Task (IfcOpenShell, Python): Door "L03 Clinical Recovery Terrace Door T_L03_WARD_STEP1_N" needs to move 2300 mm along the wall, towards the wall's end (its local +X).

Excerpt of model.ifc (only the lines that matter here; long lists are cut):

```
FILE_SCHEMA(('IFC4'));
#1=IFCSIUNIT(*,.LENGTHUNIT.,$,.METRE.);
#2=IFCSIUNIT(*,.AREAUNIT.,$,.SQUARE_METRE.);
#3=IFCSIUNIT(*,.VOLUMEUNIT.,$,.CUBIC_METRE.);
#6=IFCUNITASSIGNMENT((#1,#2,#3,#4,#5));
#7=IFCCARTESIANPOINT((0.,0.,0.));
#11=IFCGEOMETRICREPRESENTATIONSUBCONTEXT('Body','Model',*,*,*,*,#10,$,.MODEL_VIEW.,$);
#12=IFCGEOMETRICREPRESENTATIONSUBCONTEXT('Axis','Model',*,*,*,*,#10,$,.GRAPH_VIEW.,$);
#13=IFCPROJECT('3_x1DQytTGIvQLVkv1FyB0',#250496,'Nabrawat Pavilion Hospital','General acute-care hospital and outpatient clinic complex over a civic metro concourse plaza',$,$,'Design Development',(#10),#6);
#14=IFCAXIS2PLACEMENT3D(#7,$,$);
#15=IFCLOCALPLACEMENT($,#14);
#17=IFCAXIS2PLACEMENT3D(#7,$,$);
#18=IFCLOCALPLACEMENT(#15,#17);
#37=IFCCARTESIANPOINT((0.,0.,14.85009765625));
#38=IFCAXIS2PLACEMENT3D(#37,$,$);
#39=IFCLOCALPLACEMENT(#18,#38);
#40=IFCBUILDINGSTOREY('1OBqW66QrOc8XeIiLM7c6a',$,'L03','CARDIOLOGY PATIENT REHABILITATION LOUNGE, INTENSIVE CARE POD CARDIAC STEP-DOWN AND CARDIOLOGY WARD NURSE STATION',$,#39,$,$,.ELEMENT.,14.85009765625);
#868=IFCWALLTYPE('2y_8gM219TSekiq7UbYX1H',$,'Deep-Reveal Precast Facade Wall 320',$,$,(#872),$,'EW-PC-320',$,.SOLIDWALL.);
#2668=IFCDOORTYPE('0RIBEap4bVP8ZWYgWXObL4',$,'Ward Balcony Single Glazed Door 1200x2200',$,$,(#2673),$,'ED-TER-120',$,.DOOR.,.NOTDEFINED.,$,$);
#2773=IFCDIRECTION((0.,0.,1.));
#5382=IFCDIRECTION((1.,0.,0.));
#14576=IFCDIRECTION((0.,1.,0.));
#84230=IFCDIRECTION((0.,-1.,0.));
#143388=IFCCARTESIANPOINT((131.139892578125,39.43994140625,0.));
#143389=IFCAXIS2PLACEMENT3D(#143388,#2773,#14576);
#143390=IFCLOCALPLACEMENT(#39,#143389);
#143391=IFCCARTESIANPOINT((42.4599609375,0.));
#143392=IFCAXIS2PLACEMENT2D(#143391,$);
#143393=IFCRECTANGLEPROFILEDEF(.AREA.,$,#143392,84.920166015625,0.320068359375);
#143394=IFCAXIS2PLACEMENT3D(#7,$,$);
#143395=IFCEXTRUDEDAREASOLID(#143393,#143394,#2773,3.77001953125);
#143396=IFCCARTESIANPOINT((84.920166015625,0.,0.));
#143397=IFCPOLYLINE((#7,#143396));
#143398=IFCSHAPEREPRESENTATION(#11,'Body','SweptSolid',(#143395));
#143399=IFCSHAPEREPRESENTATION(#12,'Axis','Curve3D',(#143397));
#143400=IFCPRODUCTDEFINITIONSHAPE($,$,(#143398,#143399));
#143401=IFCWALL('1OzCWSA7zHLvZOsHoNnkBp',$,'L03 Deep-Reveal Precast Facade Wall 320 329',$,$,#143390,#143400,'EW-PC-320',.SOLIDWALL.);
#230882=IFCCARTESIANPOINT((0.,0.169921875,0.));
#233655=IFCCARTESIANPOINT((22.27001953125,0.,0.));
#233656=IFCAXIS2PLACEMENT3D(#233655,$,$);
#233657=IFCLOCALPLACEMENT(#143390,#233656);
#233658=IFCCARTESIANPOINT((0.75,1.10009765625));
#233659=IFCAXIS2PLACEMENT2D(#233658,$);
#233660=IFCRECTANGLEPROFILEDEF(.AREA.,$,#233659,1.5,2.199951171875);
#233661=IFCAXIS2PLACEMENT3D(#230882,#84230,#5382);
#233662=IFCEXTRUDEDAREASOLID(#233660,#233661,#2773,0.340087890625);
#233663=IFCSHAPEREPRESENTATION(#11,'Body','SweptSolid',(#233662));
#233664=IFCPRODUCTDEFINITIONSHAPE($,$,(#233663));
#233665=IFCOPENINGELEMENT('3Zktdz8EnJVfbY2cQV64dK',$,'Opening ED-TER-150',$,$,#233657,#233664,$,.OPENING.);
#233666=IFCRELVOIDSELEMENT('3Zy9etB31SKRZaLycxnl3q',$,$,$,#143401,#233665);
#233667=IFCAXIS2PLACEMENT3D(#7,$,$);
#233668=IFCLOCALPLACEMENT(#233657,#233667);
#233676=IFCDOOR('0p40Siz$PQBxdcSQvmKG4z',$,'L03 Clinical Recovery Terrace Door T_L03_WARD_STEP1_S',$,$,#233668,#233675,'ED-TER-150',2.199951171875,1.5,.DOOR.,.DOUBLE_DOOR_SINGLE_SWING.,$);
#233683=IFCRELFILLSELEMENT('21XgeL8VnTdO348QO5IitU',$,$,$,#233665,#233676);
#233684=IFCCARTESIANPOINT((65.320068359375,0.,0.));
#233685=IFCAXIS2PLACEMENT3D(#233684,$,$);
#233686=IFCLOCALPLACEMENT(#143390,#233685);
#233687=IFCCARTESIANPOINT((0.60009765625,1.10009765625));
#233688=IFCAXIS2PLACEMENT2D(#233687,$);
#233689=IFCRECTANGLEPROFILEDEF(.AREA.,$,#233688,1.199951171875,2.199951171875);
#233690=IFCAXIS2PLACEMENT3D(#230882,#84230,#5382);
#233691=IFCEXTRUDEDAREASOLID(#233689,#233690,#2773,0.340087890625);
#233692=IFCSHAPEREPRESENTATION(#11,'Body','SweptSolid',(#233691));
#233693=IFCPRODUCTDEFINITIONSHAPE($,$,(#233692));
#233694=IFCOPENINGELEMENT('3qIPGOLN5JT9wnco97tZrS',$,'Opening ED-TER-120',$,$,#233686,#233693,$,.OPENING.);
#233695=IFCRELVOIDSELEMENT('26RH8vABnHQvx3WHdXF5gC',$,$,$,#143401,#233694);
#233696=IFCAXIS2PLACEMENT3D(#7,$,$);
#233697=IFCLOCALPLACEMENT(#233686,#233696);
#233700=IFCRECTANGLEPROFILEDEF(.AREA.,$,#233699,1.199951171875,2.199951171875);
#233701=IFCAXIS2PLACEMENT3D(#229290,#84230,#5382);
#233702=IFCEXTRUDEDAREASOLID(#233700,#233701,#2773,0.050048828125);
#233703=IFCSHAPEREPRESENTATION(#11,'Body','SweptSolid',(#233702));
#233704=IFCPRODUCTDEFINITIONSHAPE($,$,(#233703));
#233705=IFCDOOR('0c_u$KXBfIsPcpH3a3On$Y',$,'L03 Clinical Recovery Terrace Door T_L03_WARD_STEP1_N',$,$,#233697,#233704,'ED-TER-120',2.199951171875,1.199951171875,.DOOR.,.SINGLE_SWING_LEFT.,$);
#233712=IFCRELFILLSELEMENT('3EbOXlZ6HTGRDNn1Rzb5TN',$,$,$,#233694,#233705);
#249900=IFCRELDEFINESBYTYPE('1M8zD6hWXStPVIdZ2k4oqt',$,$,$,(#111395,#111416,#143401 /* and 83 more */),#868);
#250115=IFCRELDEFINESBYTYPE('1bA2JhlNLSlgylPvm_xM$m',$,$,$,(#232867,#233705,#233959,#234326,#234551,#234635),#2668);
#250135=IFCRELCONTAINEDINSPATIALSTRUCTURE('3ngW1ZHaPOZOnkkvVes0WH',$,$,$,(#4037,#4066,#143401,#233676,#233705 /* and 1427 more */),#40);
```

```python
import ifcopenshell
import ifcopenshell.api.geometry
import ifcopenshell.util.placement
import ifcopenshell.util.unit

model = ifcopenshell.open("model.ifc")
unit_scale = ifcopenshell.util.unit.calculate_unit_scale(model)

door = model.by_id(233705)
opening = door.FillsVoids[0].RelatingOpeningElement
wall = opening.VoidsElements[0].RelatingBuildingElement

wall_matrix = ifcopenshell.util.placement.get_local_placement(wall.ObjectPlacement)
shift = wall_matrix[:3, 0] * 2.3 / unit_scale
before = ifcopenshell.util.placement.get_local_placement(door.ObjectPlacement)[:3, 3].copy()

# The door is placed relative to its opening, so it follows when the opening moves.
matrix = ifcopenshell.util.placement.get_local_placement(opening.ObjectPlacement)
matrix[:3, 3] += shift
ifcopenshell.api.geometry.edit_object_placement(
    model, product=opening, matrix=matrix, is_si=False, should_transform_children=True
)

after = ifcopenshell.util.placement.get_local_placement(door.ObjectPlacement)[:3, 3]
print("door moved by", (after - before).round(3) + 0.0)

model.write("model-out.ifc")
```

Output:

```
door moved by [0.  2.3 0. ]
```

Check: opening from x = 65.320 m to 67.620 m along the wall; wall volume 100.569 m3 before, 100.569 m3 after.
